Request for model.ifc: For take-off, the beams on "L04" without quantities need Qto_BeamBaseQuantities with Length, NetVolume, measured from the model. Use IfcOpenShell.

First a look at what the model holds.

```python
import ifcopenshell
import ifcopenshell.util.element
import ifcopenshell.util.unit

model = ifcopenshell.open("model.ifc")
print(model.schema)
for unit_type in ("LENGTHUNIT", "AREAUNIT", "VOLUMEUNIT"):
    print(unit_type, ifcopenshell.util.unit.calculate_unit_scale(model, unit_type))
storey = next(s for s in model.by_type("IfcBuildingStorey") if s.Name == "L04")
beams = [e for e in ifcopenshell.util.element.get_decomposition(storey) if e.is_a("IfcBeam")]
for e in sorted(beams, key=lambda e: e.id()):
    print(e.id(), e.is_a(), e.Name, list(ifcopenshell.util.element.get_psets(e, qtos_only=True)), sep=" | ")
```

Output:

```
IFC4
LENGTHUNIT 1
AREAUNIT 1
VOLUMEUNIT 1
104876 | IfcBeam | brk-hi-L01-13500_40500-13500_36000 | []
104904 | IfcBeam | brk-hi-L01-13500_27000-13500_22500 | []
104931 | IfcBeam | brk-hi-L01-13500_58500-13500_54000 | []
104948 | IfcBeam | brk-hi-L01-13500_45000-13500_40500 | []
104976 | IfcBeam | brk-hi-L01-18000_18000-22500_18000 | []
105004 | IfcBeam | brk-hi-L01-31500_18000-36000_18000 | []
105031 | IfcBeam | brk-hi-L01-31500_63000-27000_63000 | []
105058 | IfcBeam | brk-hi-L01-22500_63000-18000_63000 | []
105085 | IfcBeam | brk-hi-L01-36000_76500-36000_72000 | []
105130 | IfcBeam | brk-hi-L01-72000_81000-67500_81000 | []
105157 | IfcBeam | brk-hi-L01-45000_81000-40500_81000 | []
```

```python
import ifcopenshell
import ifcopenshell.api.pset
import ifcopenshell.geom
import ifcopenshell.util.element
import ifcopenshell.util.shape
import ifcopenshell.util.unit

model = ifcopenshell.open("model.ifc")
unit_scale = ifcopenshell.util.unit.calculate_unit_scale(model)
volume_scale = ifcopenshell.util.unit.calculate_unit_scale(model, "VOLUMEUNIT")
settings = ifcopenshell.geom.settings()

storey = next(s for s in model.by_type("IfcBuildingStorey") if s.Name == "L04")
beams = [e for e in ifcopenshell.util.element.get_decomposition(storey) if e.is_a("IfcBeam")]

for e in sorted(beams, key=lambda e: e.id()):
    if ifcopenshell.util.element.get_psets(e, qtos_only=True, should_inherit=False):
        continue
    # Geometry comes back in metres, in the element's own axes.
    shape = ifcopenshell.geom.create_shape(settings, e)
    values = {
        "Length": ifcopenshell.util.shape.get_max_xyz(shape.geometry) / unit_scale,
        "NetVolume": ifcopenshell.util.shape.get_volume(shape.geometry) / volume_scale,
    }
    qto = ifcopenshell.api.pset.add_qto(model, product=e, name="Qto_BeamBaseQuantities")
    ifcopenshell.api.pset.edit_qto(model, qto=qto, properties=values)
    print(e.id(), {k: round(v, 3) for k, v in values.items()})

model.write("model_rev.ifc")
```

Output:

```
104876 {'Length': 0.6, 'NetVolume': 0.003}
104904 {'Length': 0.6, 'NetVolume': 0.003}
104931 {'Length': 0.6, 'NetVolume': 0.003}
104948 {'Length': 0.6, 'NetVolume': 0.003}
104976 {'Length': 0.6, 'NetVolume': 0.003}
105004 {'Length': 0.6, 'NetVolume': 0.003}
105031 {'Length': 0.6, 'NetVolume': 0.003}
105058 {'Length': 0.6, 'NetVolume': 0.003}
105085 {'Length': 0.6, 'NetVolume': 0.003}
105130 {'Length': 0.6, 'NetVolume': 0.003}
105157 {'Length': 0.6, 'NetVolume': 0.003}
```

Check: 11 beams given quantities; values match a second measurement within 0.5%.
